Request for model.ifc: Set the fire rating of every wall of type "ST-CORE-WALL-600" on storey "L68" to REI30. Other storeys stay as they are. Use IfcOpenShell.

First a look at what the model holds.

```python
import ifcopenshell
import ifcopenshell.util.element

model = ifcopenshell.open("model.ifc")
print(model.schema)
storey = next(s for s in model.by_type("IfcBuildingStorey") if s.Name == "L68")
walls = [e for e in ifcopenshell.util.element.get_decomposition(storey) if e.is_a("IfcWall")]
seen = {}
for e in walls:
    element_type = ifcopenshell.util.element.get_type(e)
    key = (element_type.Name if element_type != e and element_type else None, ifcopenshell.util.element.get_pset(e, "Pset_WallCommon", "FireRating"))
    seen[key] = seen.get(key, 0) + 1
for (name, value), count in sorted(seen.items(), key=str):
    print(count, "x", name, "|", value)
```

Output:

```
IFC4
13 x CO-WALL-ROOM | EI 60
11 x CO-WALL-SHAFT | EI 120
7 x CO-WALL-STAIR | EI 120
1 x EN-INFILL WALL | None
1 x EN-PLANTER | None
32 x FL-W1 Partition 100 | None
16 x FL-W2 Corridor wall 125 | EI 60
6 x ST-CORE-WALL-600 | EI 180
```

```python
import ifcopenshell
import ifcopenshell.api.pset
import ifcopenshell.util.element

model = ifcopenshell.open("model.ifc")

storey = next(s for s in model.by_type("IfcBuildingStorey") if s.Name == "L68")
walls = [e for e in ifcopenshell.util.element.get_decomposition(storey) if e.is_a("IfcWall")]

count = 0
for e in walls:
    element_type = ifcopenshell.util.element.get_type(e)
    if element_type in (None, e) or element_type.Name != "ST-CORE-WALL-600":
        continue
    found = ifcopenshell.util.element.get_pset(e, "Pset_WallCommon", should_inherit=False)
    if found:
        pset = model.by_id(found["id"])
        if len(ifcopenshell.util.element.get_elements_by_pset(pset)) > 1:
            pset = ifcopenshell.api.pset.unshare_pset(model, products=[e], pset=pset)[0]
    else:
        pset = ifcopenshell.api.pset.add_pset(model, product=e, name="Pset_WallCommon")
    ifcopenshell.api.pset.edit_pset(model, pset=pset, properties={"FireRating": "REI30"})
    count += 1

print(count, "walls updated")

model.write("model_v2.ifc")
```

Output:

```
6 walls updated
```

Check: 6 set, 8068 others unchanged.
